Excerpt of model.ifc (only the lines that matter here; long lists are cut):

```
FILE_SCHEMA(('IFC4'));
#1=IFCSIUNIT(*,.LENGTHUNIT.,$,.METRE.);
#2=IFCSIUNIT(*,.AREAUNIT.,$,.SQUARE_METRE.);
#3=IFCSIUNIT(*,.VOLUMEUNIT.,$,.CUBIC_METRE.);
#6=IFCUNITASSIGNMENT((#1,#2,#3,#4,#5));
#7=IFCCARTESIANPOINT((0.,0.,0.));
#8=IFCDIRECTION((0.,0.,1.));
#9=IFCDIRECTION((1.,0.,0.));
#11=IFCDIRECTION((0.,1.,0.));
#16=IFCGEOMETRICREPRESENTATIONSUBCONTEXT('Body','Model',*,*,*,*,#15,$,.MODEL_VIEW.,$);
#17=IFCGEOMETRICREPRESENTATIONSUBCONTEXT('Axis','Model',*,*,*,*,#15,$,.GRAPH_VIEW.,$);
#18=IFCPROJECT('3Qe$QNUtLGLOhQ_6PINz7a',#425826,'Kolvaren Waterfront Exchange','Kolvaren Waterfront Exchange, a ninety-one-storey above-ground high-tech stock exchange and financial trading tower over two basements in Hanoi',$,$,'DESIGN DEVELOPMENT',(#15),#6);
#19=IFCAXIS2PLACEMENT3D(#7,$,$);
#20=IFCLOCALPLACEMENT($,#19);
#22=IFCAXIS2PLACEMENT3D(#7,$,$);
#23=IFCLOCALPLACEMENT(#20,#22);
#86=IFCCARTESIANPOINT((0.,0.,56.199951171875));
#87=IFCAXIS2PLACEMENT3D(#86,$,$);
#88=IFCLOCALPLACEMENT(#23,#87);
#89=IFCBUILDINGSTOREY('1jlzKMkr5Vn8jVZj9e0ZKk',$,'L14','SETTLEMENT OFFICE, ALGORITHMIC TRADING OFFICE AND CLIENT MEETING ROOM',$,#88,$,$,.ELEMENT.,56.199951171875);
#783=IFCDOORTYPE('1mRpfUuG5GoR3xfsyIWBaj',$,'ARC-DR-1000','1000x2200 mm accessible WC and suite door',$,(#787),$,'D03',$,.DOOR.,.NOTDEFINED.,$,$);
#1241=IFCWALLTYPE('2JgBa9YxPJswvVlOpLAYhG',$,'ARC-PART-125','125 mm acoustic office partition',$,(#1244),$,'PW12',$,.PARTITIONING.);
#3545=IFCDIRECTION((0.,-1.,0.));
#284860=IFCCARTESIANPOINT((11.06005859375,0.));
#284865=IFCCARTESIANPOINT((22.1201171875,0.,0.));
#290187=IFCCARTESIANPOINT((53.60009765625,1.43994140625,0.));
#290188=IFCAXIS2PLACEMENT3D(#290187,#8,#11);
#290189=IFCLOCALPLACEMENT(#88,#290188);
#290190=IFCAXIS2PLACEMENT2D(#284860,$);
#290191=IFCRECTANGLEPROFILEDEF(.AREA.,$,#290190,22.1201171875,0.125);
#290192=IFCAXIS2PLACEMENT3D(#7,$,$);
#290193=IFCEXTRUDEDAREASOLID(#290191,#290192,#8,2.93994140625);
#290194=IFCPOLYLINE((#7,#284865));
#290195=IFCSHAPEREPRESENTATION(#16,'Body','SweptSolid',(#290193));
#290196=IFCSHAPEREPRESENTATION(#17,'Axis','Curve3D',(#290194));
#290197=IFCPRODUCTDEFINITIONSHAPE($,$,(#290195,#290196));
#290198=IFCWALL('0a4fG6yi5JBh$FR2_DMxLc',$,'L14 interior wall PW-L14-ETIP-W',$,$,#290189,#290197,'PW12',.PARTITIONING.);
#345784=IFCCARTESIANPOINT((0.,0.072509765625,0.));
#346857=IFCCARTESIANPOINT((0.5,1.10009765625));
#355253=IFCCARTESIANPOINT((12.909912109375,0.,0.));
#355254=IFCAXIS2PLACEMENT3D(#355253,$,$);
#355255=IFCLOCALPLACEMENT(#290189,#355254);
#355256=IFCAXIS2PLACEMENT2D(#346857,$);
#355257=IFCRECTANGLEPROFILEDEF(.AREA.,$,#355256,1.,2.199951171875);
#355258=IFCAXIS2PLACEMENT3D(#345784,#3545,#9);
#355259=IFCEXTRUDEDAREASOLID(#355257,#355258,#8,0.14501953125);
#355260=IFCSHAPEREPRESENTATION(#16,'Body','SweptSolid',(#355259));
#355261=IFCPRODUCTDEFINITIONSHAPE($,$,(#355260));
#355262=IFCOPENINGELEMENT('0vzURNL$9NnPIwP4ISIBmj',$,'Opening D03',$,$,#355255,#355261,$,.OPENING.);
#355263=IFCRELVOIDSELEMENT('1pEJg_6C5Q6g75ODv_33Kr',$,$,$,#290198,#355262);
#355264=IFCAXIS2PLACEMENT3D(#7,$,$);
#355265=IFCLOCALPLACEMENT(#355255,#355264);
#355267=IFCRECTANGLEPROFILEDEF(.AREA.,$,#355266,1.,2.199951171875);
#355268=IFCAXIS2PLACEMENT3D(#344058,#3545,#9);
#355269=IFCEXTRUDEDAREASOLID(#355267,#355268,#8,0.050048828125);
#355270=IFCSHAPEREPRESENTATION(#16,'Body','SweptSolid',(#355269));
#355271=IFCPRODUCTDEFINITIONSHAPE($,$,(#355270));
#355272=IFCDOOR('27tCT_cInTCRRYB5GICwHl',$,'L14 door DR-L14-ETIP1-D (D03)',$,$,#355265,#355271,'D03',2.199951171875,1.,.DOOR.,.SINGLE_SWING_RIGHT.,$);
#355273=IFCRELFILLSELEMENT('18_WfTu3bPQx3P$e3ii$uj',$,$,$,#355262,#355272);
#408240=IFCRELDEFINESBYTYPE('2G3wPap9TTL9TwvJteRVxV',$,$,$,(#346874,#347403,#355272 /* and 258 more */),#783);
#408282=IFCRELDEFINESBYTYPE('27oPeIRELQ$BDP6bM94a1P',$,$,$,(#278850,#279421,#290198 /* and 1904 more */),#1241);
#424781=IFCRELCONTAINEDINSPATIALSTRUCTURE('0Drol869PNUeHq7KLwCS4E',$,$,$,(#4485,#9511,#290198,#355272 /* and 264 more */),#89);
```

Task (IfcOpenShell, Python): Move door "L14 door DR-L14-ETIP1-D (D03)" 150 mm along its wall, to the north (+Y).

```python
import ifcopenshell
import ifcopenshell.api.geometry
import ifcopenshell.util.placement

model = ifcopenshell.open("model.ifc")

door = model.by_id(355272)
opening = door.FillsVoids[0].RelatingOpeningElement
wall = opening.VoidsElements[0].RelatingBuildingElement

wall_matrix = ifcopenshell.util.placement.get_local_placement(wall.ObjectPlacement)
shift = wall_matrix[:3, 0] * 0.15
before = ifcopenshell.util.placement.get_local_placement(door.ObjectPlacement)[:3, 3].copy()

# The door is placed relative to its opening, so it follows when the opening moves.
matrix = ifcopenshell.util.placement.get_local_placement(opening.ObjectPlacement)
matrix[:3, 3] += shift
ifcopenshell.api.geometry.edit_object_placement(
    model, product=opening, matrix=matrix, is_si=False, should_transform_children=True
)

after = ifcopenshell.util.placement.get_local_placement(door.ObjectPlacement)[:3, 3]
print("door moved by", (after - before).round(3) + 0.0)

model.write("model_updated.ifc")
```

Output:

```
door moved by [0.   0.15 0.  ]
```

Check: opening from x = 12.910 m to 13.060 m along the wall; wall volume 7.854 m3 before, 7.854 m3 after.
